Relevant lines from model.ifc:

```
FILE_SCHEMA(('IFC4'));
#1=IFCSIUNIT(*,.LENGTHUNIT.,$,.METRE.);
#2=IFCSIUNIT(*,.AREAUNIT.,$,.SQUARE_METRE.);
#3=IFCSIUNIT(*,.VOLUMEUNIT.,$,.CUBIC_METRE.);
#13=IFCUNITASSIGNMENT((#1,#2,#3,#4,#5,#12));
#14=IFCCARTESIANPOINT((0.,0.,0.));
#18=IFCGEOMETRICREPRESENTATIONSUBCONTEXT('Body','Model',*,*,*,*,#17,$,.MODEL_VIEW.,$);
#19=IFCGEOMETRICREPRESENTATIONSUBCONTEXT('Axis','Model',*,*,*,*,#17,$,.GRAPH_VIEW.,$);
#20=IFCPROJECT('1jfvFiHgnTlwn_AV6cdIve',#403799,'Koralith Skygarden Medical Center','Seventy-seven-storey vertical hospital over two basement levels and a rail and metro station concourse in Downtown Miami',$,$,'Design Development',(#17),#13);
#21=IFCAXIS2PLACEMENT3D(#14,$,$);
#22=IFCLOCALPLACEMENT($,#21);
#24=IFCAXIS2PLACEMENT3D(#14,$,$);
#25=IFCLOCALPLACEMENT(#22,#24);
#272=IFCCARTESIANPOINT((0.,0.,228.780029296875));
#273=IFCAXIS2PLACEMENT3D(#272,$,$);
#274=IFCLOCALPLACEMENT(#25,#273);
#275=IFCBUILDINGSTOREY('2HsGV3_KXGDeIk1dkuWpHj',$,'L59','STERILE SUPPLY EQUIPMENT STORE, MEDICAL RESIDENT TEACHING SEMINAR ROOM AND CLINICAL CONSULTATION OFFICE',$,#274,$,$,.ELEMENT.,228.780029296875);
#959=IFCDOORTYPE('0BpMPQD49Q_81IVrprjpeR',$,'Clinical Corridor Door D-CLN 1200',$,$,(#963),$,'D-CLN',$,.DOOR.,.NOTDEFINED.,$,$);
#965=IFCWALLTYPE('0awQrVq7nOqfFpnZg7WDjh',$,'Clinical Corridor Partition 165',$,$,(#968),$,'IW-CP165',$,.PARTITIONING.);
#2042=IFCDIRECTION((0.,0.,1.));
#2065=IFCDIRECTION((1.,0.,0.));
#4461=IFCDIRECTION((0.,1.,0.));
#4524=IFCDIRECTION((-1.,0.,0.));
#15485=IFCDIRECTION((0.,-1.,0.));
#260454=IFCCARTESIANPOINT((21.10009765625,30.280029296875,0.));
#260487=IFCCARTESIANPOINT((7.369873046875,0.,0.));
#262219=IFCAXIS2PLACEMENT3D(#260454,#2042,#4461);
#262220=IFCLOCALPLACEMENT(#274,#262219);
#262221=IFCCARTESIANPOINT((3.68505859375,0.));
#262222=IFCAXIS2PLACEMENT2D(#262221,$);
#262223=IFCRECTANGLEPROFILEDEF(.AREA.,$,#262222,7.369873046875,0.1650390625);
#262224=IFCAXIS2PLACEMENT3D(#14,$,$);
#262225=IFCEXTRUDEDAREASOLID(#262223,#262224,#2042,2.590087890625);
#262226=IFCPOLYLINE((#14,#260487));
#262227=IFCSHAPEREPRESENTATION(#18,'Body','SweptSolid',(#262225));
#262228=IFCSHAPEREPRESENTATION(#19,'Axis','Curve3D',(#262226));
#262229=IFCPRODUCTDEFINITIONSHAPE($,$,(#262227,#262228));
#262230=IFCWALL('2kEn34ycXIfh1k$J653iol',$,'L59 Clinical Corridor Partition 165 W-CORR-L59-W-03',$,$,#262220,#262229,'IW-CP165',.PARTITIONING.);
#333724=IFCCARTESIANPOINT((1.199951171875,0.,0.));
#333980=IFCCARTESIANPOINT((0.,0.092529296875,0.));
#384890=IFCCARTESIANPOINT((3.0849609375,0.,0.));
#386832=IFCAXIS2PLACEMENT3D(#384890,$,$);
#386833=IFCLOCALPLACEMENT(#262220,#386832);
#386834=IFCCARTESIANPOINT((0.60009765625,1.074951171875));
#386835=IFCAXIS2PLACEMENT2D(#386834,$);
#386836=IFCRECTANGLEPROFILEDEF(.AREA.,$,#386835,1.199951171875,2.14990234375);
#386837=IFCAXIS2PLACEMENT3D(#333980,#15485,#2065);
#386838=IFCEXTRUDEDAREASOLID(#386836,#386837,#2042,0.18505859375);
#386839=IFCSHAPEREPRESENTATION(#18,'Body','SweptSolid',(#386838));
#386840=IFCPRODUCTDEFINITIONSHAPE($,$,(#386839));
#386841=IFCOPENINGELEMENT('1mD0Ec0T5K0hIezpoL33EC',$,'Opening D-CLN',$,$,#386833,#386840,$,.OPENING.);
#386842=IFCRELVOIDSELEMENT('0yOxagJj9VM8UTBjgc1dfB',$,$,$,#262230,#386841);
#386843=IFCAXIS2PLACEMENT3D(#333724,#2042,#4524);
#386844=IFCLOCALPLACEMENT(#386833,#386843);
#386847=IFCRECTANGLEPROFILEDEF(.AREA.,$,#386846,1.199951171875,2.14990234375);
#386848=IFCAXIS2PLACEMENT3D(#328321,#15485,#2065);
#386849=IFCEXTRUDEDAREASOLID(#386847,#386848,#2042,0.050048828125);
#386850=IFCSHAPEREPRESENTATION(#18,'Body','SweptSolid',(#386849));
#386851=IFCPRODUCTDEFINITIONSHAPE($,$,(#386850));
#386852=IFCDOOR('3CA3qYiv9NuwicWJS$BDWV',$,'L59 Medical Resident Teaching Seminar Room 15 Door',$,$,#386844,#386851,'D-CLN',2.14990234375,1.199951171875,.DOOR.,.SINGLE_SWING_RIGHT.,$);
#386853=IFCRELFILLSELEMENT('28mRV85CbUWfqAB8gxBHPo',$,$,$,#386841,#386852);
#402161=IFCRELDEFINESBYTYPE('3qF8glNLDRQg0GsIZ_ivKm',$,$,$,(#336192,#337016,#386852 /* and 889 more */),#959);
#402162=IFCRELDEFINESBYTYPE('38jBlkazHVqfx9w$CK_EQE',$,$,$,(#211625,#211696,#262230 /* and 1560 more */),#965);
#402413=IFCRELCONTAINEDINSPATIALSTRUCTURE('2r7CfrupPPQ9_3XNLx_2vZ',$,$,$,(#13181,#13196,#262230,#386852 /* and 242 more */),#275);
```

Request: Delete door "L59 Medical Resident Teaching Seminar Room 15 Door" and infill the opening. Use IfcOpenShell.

```python
import ifcopenshell
import ifcopenshell.api.feature
import ifcopenshell.api.root
import ifcopenshell.geom
import ifcopenshell.util.shape

model = ifcopenshell.open("model.ifc")
settings = ifcopenshell.geom.settings()


def volume(element):
    """Net volume in cubic metres, openings subtracted."""
    shape = ifcopenshell.geom.create_shape(settings, element)
    return ifcopenshell.util.shape.get_volume(shape.geometry)


door = model.by_guid("3CA3qYiv9NuwicWJS$BDWV")
opening = door.FillsVoids[0].RelatingOpeningElement
wall = opening.VoidsElements[0].RelatingBuildingElement
before = volume(wall)

ifcopenshell.api.root.remove_product(model, product=door)
ifcopenshell.api.feature.remove_feature(model, feature=opening)

after = volume(wall)

print(f"wall volume {before:.3f} -> {after:.3f} m3")

model.write("model_v2.ifc")
```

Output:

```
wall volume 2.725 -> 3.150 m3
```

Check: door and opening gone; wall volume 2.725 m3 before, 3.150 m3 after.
